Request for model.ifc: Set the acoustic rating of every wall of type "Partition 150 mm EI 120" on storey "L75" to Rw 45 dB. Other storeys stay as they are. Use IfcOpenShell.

First a look at what the model holds.

```python
import ifcopenshell
import ifcopenshell.util.element

model = ifcopenshell.open("model.ifc")
print(model.schema)
storey = next(s for s in model.by_type("IfcBuildingStorey") if s.Name == "L75")
walls = [e for e in ifcopenshell.util.element.get_decomposition(storey) if e.is_a("IfcWall")]
seen = {}
for e in walls:
    element_type = ifcopenshell.util.element.get_type(e)
    key = (element_type.Name if element_type != e and element_type else None, ifcopenshell.util.element.get_pset(e, "Pset_WallCommon", "AcousticRating"))
    seen[key] = seen.get(key, 0) + 1
for (name, value), count in sorted(seen.items(), key=str):
    print(count, "x", name, "|", value)
```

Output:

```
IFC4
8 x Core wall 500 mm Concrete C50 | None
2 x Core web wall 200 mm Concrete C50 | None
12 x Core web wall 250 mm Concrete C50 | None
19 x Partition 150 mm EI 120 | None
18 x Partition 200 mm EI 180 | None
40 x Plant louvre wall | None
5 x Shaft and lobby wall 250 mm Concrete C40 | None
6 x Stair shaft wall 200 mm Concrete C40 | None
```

```python
import ifcopenshell
import ifcopenshell.api.pset
import ifcopenshell.util.element

model = ifcopenshell.open("model.ifc")

storey = next(s for s in model.by_type("IfcBuildingStorey") if s.Name == "L75")
walls = [e for e in ifcopenshell.util.element.get_decomposition(storey) if e.is_a("IfcWall")]

count = 0
for e in walls:
    element_type = ifcopenshell.util.element.get_type(e)
    if element_type in (None, e) or element_type.Name != "Partition 150 mm EI 120":
        continue
    found = ifcopenshell.util.element.get_pset(e, "Pset_WallCommon", should_inherit=False)
    if found:
        pset = model.by_id(found["id"])
        if len(ifcopenshell.util.element.get_elements_by_pset(pset)) > 1:
            pset = ifcopenshell.api.pset.unshare_pset(model, products=[e], pset=pset)[0]
    else:
        pset = ifcopenshell.api.pset.add_pset(model, product=e, name="Pset_WallCommon")
    ifcopenshell.api.pset.edit_pset(model, pset=pset, properties={"AcousticRating": "Rw 45 dB"})
    count += 1

print(count, "walls updated")

model.write("model-out.ifc")
```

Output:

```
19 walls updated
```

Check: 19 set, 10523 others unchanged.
